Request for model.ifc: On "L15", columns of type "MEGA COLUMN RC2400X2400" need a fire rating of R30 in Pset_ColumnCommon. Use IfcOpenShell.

First a look at what the model holds.

```python
import ifcopenshell
import ifcopenshell.util.element

model = ifcopenshell.open("model.ifc")
print(model.schema)
storey = next(s for s in model.by_type("IfcBuildingStorey") if s.Name == "L15")
columns = [e for e in ifcopenshell.util.element.get_decomposition(storey) if e.is_a("IfcColumn")]
seen = {}
for e in columns:
    element_type = ifcopenshell.util.element.get_type(e)
    key = (element_type.Name if element_type != e and element_type else None, ifcopenshell.util.element.get_pset(e, "Pset_ColumnCommon", "FireRating"))
    seen[key] = seen.get(key, 0) + 1
for (name, value), count in sorted(seen.items(), key=str):
    print(count, "x", name, "|", value)
```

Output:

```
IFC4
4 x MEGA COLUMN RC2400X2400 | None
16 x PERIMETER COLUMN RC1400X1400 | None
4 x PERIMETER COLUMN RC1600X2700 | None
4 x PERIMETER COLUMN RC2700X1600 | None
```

```python
import ifcopenshell
import ifcopenshell.api.pset
import ifcopenshell.util.element

model = ifcopenshell.open("model.ifc")

storey = next(s for s in model.by_type("IfcBuildingStorey") if s.Name == "L15")
columns = [e for e in ifcopenshell.util.element.get_decomposition(storey) if e.is_a("IfcColumn")]

count = 0
for e in columns:
    element_type = ifcopenshell.util.element.get_type(e)
    if element_type in (None, e) or element_type.Name != "MEGA COLUMN RC2400X2400":
        continue
    found = ifcopenshell.util.element.get_pset(e, "Pset_ColumnCommon", should_inherit=False)
    if found:
        pset = model.by_id(found["id"])
        if len(ifcopenshell.util.element.get_elements_by_pset(pset)) > 1:
            pset = ifcopenshell.api.pset.unshare_pset(model, products=[e], pset=pset)[0]
    else:
        pset = ifcopenshell.api.pset.add_pset(model, product=e, name="Pset_ColumnCommon")
    ifcopenshell.api.pset.edit_pset(model, pset=pset, properties={"FireRating": "R30"})
    count += 1

print(count, "columns updated")

model.write("model_updated.ifc")
```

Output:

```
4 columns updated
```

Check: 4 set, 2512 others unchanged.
